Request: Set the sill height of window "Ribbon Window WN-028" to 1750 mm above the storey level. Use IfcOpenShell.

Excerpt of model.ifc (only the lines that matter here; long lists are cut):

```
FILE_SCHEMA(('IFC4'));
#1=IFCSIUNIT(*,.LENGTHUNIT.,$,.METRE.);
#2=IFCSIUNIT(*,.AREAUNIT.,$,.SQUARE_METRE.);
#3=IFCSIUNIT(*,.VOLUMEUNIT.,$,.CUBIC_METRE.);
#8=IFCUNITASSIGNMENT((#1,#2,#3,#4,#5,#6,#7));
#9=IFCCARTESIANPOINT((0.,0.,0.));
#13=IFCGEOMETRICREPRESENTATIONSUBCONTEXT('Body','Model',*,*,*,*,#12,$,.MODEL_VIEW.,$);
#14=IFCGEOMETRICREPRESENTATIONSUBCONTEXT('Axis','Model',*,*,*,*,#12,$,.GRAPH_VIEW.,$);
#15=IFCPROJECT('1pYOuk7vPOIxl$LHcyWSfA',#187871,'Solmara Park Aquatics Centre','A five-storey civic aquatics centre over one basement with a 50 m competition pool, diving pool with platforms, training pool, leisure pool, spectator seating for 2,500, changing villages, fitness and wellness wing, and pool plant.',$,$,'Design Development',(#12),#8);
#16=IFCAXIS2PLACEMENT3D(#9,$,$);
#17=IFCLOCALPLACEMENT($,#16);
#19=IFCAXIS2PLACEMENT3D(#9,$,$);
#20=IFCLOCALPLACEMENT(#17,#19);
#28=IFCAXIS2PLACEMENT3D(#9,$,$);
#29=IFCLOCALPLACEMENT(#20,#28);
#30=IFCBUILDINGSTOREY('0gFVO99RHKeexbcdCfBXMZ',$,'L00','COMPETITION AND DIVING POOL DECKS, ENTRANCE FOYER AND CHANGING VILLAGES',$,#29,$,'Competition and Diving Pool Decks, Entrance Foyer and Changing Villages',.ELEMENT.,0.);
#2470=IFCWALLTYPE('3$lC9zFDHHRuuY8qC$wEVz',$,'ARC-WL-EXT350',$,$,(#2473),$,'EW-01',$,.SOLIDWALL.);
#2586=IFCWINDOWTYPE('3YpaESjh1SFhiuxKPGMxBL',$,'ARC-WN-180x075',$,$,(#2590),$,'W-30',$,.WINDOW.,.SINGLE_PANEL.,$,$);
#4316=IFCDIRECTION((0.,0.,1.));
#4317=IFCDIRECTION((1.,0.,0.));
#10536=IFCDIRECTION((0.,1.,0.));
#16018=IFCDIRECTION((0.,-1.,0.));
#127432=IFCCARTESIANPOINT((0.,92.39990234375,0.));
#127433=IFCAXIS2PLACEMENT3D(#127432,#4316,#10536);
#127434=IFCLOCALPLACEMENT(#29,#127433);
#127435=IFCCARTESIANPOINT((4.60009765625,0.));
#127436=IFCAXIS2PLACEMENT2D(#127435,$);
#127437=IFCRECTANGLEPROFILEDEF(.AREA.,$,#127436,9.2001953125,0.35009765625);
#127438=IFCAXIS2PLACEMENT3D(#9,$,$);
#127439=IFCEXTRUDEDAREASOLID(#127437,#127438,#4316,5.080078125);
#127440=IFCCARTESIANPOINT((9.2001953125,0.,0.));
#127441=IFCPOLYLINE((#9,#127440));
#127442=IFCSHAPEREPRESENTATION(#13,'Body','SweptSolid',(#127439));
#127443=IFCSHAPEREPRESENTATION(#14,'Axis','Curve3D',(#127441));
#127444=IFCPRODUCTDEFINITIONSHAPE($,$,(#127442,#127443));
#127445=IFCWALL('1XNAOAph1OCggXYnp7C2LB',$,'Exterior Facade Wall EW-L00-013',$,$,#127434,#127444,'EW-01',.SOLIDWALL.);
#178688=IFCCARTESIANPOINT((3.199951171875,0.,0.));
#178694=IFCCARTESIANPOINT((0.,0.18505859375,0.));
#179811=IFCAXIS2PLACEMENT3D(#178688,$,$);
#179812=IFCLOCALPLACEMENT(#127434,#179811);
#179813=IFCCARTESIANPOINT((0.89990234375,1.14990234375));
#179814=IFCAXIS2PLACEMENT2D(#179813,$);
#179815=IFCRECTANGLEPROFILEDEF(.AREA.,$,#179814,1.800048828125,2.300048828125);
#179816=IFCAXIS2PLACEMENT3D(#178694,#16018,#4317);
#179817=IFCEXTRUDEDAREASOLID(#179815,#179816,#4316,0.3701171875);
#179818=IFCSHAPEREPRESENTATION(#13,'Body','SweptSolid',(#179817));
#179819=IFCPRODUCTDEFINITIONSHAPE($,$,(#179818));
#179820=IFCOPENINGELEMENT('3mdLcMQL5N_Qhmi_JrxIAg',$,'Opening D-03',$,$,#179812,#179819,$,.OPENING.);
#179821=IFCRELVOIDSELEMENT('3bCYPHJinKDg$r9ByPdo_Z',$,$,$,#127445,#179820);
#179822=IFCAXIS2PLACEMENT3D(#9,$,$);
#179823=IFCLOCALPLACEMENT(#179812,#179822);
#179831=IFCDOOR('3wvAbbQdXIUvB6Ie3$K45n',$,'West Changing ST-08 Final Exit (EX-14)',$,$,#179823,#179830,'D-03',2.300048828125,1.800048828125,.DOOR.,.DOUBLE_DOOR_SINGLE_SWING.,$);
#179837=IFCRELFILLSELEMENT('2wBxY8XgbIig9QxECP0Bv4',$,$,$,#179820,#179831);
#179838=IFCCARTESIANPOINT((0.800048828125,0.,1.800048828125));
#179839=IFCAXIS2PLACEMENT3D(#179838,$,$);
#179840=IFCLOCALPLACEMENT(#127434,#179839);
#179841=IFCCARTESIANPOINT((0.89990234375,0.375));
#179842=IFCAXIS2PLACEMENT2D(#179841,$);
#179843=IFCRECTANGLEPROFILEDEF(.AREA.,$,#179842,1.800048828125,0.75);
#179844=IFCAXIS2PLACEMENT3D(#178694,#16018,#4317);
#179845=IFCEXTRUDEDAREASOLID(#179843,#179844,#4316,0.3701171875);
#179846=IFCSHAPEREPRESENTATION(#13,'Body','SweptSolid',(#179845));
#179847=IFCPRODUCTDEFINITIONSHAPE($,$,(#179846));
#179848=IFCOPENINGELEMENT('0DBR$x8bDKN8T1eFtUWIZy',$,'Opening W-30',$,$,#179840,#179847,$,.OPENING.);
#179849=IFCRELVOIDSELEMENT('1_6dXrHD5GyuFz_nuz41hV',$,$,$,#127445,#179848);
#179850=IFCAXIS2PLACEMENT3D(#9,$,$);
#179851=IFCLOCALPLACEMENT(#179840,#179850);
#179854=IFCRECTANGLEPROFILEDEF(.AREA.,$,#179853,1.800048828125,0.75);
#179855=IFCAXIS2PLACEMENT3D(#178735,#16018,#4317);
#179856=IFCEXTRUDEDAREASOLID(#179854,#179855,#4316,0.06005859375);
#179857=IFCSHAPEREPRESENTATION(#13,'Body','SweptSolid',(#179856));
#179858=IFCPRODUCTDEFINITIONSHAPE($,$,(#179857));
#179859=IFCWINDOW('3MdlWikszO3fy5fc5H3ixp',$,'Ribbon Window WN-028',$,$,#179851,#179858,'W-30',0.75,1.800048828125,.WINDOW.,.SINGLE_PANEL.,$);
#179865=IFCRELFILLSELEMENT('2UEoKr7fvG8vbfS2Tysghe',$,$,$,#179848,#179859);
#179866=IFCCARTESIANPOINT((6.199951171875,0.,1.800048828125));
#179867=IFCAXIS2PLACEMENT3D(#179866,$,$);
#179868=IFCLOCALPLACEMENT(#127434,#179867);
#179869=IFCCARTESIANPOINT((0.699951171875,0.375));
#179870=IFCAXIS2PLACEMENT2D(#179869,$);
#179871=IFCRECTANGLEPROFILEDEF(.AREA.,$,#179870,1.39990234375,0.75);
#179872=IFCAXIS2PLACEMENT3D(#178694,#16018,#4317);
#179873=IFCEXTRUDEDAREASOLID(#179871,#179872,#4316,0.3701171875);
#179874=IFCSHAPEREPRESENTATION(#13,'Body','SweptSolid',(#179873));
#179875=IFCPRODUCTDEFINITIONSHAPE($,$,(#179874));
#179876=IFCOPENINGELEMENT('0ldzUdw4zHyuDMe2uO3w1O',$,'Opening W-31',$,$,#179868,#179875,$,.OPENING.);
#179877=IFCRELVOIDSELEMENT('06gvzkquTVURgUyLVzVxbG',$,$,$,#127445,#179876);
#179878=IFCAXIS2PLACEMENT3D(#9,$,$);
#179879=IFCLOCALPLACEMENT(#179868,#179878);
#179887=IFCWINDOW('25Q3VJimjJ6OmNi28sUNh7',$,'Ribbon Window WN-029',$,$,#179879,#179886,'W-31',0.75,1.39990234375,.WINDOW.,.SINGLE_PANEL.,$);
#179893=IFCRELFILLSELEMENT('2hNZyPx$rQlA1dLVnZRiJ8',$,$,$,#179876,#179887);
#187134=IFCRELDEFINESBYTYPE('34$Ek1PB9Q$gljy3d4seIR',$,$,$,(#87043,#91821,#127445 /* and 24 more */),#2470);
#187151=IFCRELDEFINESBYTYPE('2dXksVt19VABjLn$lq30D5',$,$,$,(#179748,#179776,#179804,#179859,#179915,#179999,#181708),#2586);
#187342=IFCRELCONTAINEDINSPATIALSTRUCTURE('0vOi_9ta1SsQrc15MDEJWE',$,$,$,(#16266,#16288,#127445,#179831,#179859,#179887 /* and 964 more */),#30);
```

```python
import numpy as np
import ifcopenshell
import ifcopenshell.api.geometry
import ifcopenshell.geom
import ifcopenshell.util.element
import ifcopenshell.util.placement
import ifcopenshell.util.shape
import ifcopenshell.util.unit

model = ifcopenshell.open("model.ifc")
unit_scale = ifcopenshell.util.unit.calculate_unit_scale(model)

window = model.by_id(179859)
opening = window.FillsVoids[0].RelatingOpeningElement
storey = ifcopenshell.util.element.get_container(window, ifc_class="IfcBuildingStorey")
level = ifcopenshell.util.placement.get_local_placement(storey.ObjectPlacement)[2, 3]

# The opening's origin need not be at the sill, so measure its lowest point.
shape = ifcopenshell.geom.create_shape(ifcopenshell.geom.settings(), opening)
bottom = ifcopenshell.util.shape.get_shape_bottom_elevation(shape, shape.geometry) / unit_scale
dz = level + 1.75 - bottom

shift = np.array([0.0, 0.0, dz])
# The window is placed relative to its opening, so it follows when the opening moves.
matrix = ifcopenshell.util.placement.get_local_placement(opening.ObjectPlacement)
matrix[:3, 3] += shift
ifcopenshell.api.geometry.edit_object_placement(
    model, product=opening, matrix=matrix, is_si=False, should_transform_children=True
)

print(f"moved by {dz * unit_scale:+.3f} m")

model.write("model-out.ifc")
```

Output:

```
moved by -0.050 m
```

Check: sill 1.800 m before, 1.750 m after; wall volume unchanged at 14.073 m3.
